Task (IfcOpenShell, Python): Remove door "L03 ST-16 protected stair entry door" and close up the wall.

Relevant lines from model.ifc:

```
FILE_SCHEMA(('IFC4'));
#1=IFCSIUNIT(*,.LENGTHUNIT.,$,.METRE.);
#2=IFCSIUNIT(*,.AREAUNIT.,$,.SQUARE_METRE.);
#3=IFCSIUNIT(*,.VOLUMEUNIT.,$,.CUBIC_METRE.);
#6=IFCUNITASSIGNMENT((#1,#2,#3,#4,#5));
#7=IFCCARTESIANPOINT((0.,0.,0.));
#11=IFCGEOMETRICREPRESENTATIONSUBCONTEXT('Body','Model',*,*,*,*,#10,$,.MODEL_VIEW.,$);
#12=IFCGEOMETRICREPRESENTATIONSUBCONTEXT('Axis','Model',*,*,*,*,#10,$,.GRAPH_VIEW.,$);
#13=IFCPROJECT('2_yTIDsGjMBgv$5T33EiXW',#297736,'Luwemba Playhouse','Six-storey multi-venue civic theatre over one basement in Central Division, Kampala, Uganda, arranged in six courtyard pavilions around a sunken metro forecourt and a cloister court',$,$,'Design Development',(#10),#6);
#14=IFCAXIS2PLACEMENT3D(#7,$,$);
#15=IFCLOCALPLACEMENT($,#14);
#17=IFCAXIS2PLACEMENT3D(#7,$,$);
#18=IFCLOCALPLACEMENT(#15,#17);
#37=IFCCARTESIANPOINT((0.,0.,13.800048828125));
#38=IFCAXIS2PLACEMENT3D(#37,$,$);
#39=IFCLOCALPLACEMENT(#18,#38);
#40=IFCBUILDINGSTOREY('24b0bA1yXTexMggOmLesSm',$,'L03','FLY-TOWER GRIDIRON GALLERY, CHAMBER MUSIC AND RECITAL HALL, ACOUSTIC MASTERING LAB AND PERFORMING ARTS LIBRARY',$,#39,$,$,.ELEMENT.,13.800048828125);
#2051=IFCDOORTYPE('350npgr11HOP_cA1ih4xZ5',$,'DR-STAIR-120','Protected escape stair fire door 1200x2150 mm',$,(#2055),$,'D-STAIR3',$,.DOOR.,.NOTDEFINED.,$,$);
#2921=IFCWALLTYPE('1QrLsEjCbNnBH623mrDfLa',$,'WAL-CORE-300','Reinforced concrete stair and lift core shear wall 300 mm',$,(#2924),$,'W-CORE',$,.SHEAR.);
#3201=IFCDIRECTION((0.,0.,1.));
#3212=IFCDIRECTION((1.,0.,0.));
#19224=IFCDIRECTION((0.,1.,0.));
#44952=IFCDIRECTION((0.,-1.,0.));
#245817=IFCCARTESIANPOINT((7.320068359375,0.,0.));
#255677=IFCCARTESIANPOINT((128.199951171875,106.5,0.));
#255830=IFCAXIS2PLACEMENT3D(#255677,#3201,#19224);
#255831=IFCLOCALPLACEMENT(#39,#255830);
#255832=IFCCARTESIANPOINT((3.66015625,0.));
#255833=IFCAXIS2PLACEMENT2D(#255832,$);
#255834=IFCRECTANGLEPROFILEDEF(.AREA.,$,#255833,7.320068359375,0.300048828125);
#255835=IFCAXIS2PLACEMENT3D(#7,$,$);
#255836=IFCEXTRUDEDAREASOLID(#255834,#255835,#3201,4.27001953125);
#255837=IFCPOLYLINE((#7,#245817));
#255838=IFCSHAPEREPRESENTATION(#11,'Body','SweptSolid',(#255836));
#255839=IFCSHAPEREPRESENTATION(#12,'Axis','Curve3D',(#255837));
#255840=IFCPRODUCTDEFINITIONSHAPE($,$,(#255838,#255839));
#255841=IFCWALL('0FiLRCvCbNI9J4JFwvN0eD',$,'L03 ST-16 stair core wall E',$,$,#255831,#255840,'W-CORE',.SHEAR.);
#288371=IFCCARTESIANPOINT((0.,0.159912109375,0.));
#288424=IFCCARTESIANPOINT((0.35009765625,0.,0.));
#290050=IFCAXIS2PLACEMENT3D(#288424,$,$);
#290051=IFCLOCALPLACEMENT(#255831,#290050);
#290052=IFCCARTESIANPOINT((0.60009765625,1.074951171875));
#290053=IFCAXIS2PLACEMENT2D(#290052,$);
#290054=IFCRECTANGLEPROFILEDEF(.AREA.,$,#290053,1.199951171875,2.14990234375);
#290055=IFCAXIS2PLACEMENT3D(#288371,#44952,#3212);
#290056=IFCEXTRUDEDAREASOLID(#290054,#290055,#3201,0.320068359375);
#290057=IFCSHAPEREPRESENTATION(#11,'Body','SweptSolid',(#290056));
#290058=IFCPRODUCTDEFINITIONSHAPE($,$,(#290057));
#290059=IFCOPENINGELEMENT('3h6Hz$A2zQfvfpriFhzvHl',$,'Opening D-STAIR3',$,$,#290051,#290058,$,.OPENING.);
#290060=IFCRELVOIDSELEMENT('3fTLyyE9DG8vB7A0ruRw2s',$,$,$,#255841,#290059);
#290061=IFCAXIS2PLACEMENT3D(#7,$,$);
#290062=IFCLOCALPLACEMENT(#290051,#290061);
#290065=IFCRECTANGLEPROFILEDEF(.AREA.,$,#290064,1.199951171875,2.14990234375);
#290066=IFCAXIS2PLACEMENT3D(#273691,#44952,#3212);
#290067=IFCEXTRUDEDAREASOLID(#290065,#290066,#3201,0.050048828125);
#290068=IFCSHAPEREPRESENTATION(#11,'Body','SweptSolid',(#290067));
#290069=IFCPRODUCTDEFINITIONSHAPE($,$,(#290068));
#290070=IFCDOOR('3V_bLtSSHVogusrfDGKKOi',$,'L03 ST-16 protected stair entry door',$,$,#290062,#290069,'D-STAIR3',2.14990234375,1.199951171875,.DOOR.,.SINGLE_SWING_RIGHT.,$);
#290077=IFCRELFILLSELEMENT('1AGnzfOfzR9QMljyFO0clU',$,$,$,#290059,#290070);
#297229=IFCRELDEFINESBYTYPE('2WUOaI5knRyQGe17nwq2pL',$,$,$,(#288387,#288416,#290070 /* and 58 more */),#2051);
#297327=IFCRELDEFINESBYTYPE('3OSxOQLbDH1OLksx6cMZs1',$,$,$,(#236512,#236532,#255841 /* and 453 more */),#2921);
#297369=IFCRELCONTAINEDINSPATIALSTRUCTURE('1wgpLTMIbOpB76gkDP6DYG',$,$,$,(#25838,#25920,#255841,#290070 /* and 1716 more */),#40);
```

```python
import ifcopenshell
import ifcopenshell.api.feature
import ifcopenshell.api.root
import ifcopenshell.geom
import ifcopenshell.util.shape

model = ifcopenshell.open("model.ifc")
settings = ifcopenshell.geom.settings()


def volume(element):
    """Net volume in cubic metres, openings subtracted."""
    shape = ifcopenshell.geom.create_shape(settings, element)
    return ifcopenshell.util.shape.get_volume(shape.geometry)


door = model.by_guid("3V_bLtSSHVogusrfDGKKOi")
opening = door.FillsVoids[0].RelatingOpeningElement
wall = opening.VoidsElements[0].RelatingBuildingElement
before = volume(wall)

ifcopenshell.api.root.remove_product(model, product=door)
ifcopenshell.api.feature.remove_feature(model, feature=opening)

after = volume(wall)

print(f"wall volume {before:.3f} -> {after:.3f} m3")

model.write("model-out.ifc")
```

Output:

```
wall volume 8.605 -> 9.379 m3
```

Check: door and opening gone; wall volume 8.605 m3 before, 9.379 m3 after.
